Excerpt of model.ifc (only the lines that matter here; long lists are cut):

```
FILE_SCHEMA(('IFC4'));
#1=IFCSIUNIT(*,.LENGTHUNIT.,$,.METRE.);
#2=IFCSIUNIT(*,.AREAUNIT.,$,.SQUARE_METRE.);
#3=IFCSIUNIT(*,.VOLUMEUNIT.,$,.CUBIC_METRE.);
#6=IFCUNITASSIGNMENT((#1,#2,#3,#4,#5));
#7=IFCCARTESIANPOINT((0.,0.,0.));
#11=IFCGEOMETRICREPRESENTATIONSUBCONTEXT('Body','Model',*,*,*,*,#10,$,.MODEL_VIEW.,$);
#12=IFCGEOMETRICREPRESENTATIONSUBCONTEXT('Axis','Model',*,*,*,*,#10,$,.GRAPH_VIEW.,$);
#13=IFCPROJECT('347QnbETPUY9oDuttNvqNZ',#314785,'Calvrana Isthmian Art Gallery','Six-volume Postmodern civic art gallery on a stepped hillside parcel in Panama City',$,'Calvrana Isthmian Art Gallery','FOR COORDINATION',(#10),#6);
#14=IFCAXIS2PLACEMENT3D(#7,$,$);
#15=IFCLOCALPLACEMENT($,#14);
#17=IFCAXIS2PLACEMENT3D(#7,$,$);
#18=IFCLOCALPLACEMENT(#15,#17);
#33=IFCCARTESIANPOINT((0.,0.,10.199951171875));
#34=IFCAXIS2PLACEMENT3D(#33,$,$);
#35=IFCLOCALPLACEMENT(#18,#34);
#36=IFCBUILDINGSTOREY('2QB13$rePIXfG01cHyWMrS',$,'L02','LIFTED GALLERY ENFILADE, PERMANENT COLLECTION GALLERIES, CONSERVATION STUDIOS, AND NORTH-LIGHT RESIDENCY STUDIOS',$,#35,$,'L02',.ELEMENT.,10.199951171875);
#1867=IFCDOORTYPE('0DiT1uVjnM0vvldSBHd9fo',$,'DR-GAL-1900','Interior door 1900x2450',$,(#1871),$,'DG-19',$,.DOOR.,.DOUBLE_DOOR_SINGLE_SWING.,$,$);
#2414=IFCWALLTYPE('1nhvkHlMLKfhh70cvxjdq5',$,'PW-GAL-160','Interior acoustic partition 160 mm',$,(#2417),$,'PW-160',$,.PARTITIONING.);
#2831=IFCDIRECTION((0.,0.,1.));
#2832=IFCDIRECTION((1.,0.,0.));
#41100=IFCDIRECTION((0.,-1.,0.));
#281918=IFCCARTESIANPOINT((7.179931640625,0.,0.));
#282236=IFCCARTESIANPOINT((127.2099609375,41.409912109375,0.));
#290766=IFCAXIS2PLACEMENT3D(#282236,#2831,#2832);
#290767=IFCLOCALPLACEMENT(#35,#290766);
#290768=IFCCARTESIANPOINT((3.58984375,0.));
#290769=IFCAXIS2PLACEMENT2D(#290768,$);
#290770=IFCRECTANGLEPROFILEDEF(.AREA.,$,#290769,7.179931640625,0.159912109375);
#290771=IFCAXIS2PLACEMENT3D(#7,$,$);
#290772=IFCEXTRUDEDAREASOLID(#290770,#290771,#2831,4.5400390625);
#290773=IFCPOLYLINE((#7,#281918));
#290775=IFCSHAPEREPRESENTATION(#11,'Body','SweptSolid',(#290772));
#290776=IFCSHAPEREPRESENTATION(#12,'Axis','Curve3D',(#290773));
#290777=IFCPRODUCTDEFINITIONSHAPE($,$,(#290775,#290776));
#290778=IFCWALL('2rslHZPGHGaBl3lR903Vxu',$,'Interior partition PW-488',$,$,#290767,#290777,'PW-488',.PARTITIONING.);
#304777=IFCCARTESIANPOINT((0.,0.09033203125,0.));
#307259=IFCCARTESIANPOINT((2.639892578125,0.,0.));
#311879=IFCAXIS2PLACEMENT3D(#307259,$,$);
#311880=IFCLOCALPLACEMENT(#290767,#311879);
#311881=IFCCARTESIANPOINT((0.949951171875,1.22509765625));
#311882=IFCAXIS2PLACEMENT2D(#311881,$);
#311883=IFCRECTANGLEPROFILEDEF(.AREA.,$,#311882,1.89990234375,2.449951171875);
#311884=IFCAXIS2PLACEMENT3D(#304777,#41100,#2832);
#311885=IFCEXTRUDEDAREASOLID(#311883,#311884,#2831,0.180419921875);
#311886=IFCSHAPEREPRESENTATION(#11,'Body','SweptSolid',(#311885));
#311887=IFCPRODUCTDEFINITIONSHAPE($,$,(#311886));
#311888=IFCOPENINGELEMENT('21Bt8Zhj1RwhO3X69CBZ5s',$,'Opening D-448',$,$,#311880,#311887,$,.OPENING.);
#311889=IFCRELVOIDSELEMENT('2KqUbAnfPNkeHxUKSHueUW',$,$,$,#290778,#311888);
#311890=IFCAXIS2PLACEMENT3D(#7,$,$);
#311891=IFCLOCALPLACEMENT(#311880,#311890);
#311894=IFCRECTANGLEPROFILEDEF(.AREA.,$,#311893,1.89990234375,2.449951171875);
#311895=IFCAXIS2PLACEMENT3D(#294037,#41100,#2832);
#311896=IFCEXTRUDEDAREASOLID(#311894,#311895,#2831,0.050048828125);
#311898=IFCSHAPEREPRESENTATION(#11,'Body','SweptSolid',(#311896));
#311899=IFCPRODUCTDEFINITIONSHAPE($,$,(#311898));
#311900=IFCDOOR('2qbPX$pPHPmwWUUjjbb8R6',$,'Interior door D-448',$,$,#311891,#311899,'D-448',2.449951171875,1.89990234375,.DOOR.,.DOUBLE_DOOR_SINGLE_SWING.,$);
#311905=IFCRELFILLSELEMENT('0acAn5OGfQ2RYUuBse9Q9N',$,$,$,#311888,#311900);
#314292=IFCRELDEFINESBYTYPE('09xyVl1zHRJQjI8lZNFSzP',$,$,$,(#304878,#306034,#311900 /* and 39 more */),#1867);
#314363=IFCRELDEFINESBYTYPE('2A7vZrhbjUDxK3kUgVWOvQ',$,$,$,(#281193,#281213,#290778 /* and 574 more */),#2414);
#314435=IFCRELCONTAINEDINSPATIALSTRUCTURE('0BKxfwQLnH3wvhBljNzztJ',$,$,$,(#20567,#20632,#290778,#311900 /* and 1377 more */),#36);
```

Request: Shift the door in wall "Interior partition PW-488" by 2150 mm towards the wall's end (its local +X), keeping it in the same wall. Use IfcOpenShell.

```python
import ifcopenshell
import ifcopenshell.api.geometry
import ifcopenshell.util.placement
import ifcopenshell.util.unit

model = ifcopenshell.open("model.ifc")
unit_scale = ifcopenshell.util.unit.calculate_unit_scale(model)

door = model.by_id(311900)
opening = door.FillsVoids[0].RelatingOpeningElement
wall = opening.VoidsElements[0].RelatingBuildingElement

wall_matrix = ifcopenshell.util.placement.get_local_placement(wall.ObjectPlacement)
shift = wall_matrix[:3, 0] * 2.15 / unit_scale
before = ifcopenshell.util.placement.get_local_placement(door.ObjectPlacement)[:3, 3].copy()

# The door is placed relative to its opening, so it follows when the opening moves.
matrix = ifcopenshell.util.placement.get_local_placement(opening.ObjectPlacement)
matrix[:3, 3] += shift
ifcopenshell.api.geometry.edit_object_placement(
    model, product=opening, matrix=matrix, is_si=False, should_transform_children=True
)

after = ifcopenshell.util.placement.get_local_placement(door.ObjectPlacement)[:3, 3]
print("door moved by", (after - before).round(3) + 0.0)

model.write("model_v2.ifc")
```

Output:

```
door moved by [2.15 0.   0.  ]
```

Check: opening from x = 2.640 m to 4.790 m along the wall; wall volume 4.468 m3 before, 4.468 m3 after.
